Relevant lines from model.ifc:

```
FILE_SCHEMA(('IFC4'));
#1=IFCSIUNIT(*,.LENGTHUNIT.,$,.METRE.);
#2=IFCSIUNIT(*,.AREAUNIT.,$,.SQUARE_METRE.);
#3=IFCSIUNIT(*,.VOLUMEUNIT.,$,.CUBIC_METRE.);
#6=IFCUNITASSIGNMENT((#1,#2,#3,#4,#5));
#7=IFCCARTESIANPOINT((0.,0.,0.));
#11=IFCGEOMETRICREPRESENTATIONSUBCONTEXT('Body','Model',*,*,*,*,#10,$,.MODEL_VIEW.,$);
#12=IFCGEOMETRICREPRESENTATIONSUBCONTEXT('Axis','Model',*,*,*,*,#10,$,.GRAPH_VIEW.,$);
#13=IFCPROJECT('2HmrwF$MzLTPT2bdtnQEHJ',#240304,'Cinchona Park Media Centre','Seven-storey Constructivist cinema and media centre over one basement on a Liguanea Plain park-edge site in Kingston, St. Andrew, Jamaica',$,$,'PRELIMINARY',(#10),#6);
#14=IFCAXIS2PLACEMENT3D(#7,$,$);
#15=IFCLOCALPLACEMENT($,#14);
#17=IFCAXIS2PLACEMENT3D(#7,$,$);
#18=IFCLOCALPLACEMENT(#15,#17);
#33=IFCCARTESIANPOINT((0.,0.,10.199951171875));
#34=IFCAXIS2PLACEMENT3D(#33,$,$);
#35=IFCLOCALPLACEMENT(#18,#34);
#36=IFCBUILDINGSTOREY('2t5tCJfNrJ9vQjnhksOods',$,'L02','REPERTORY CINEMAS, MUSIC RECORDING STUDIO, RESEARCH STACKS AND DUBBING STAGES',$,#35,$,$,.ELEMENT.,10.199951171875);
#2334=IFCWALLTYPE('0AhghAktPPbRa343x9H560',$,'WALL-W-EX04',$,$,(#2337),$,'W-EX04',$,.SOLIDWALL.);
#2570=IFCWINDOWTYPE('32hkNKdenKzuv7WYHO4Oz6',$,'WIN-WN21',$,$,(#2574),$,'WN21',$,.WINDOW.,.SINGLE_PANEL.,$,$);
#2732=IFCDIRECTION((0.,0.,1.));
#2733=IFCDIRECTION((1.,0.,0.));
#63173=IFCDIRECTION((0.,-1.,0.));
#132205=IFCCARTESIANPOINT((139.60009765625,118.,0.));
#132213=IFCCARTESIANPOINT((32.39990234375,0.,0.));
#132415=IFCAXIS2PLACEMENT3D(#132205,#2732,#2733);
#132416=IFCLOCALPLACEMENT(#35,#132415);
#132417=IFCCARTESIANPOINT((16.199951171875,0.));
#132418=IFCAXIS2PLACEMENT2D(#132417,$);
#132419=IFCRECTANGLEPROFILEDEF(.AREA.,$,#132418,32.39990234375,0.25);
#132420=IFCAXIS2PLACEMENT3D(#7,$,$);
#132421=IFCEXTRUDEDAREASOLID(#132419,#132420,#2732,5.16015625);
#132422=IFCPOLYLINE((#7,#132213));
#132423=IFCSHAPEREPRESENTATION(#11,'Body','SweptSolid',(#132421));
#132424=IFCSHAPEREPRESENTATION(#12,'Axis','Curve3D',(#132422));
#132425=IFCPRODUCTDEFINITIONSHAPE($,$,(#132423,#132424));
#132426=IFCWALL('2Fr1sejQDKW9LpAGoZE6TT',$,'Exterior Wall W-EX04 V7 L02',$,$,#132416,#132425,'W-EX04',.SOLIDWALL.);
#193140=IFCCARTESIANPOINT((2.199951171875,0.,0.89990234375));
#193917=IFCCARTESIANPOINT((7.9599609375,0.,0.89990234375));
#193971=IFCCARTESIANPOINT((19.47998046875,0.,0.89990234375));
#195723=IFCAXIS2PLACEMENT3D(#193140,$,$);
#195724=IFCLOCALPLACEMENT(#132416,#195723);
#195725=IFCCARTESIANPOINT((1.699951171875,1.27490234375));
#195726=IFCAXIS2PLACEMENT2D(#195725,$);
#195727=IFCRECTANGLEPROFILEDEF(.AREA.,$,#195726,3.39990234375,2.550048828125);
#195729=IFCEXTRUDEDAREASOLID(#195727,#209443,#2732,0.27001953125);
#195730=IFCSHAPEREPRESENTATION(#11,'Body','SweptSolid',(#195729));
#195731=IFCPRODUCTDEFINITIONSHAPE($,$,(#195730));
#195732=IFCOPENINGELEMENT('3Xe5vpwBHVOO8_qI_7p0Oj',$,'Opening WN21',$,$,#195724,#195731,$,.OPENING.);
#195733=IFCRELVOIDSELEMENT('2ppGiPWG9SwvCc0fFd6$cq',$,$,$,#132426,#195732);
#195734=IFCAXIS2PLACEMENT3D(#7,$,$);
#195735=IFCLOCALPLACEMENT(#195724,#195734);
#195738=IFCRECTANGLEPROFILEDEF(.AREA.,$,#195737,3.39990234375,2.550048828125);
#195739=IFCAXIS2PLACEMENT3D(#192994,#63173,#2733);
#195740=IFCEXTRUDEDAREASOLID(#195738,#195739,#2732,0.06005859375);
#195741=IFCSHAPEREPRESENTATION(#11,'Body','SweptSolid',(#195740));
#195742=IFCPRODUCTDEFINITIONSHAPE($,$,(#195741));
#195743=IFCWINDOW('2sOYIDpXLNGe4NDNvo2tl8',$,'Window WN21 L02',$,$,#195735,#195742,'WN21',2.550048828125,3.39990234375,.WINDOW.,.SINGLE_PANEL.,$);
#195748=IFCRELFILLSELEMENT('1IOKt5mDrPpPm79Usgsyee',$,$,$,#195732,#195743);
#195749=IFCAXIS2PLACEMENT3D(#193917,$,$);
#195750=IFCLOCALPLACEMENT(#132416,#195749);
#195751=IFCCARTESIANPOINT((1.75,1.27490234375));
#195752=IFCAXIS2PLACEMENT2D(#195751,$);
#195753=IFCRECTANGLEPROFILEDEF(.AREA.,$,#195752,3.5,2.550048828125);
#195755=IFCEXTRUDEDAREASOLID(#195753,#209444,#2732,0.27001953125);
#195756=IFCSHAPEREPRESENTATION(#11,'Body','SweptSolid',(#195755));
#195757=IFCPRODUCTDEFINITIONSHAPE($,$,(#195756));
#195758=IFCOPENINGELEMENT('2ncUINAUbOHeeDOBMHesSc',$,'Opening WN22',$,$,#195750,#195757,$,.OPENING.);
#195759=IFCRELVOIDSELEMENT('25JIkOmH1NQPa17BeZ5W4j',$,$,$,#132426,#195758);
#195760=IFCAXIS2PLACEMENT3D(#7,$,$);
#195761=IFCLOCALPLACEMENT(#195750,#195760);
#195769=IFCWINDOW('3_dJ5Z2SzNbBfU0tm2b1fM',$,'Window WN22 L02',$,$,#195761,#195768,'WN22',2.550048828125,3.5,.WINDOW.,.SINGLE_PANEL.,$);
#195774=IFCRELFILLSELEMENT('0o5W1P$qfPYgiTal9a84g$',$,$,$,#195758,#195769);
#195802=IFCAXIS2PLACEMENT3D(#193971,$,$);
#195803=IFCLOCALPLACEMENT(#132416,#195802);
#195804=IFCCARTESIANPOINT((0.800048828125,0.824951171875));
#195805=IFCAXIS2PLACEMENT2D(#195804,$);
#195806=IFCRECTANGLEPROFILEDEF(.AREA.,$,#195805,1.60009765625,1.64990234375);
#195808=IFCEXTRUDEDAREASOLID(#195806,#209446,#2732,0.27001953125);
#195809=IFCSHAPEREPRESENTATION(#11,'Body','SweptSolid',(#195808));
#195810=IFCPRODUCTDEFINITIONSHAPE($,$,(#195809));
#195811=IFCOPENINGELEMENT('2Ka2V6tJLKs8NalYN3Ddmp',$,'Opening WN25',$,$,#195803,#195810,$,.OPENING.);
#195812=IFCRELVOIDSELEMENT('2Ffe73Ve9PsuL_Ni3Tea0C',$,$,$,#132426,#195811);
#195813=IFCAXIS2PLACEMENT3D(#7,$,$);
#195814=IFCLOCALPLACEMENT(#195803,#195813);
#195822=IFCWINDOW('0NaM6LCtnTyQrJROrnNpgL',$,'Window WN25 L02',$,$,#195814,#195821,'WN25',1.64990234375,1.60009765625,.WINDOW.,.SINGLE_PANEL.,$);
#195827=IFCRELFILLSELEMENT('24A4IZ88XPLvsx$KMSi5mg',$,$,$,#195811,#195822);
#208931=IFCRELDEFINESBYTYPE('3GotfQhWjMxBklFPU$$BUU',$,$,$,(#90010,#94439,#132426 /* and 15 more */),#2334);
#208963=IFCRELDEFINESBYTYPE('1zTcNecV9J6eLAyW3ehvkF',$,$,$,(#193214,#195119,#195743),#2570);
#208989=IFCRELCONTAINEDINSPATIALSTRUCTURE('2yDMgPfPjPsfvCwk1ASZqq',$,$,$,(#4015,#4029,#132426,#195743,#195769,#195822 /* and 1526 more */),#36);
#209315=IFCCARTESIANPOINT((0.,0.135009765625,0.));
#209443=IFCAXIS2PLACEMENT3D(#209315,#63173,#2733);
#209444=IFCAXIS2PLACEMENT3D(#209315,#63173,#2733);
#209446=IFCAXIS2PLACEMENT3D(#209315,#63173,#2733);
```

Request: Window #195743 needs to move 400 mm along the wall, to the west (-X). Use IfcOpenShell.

```python
import ifcopenshell
import ifcopenshell.api.geometry
import ifcopenshell.util.placement
import ifcopenshell.util.unit

model = ifcopenshell.open("model.ifc")
unit_scale = ifcopenshell.util.unit.calculate_unit_scale(model)

window = model.by_guid("2sOYIDpXLNGe4NDNvo2tl8")
opening = window.FillsVoids[0].RelatingOpeningElement
wall = opening.VoidsElements[0].RelatingBuildingElement

wall_matrix = ifcopenshell.util.placement.get_local_placement(wall.ObjectPlacement)
shift = wall_matrix[:3, 0] * -0.4 / unit_scale
before = ifcopenshell.util.placement.get_local_placement(window.ObjectPlacement)[:3, 3].copy()

# The window is placed relative to its opening, so it follows when the opening moves.
matrix = ifcopenshell.util.placement.get_local_placement(opening.ObjectPlacement)
matrix[:3, 3] += shift
ifcopenshell.api.geometry.edit_object_placement(
    model, product=opening, matrix=matrix, is_si=False, should_transform_children=True
)

after = ifcopenshell.util.placement.get_local_placement(window.ObjectPlacement)[:3, 3]
print("window moved by", (after - before).round(3) + 0.0)

model.write("model_edited.ifc")
```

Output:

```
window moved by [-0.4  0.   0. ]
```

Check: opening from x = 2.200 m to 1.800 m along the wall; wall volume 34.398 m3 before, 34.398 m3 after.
